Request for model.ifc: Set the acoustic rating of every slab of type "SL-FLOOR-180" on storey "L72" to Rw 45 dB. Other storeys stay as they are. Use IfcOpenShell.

First a look at what the model holds.

```python
import ifcopenshell
import ifcopenshell.util.element

model = ifcopenshell.open("model.ifc")
print(model.schema)
storey = next(s for s in model.by_type("IfcBuildingStorey") if s.Name == "L72")
slabs = [e for e in ifcopenshell.util.element.get_decomposition(storey) if e.is_a("IfcSlab")]
seen = {}
for e in slabs:
    element_type = ifcopenshell.util.element.get_type(e)
    key = (element_type.Name if element_type != e and element_type else None, ifcopenshell.util.element.get_pset(e, "Pset_SlabCommon", "AcousticRating"))
    seen[key] = seen.get(key, 0) + 1
for (name, value), count in sorted(seen.items(), key=str):
    print(count, "x", name, "|", value)
```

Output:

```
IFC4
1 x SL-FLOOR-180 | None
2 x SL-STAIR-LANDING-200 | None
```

```python
import ifcopenshell
import ifcopenshell.api.pset
import ifcopenshell.util.element

model = ifcopenshell.open("model.ifc")

storey = next(s for s in model.by_type("IfcBuildingStorey") if s.Name == "L72")
slabs = [e for e in ifcopenshell.util.element.get_decomposition(storey) if e.is_a("IfcSlab")]

count = 0
for e in slabs:
    element_type = ifcopenshell.util.element.get_type(e)
    if element_type in (None, e) or element_type.Name != "SL-FLOOR-180":
        continue
    # add_pset returns the element's existing set when there is one.
    pset = ifcopenshell.api.pset.add_pset(model, product=e, name="Pset_SlabCommon")
    ifcopenshell.api.pset.edit_pset(model, pset=pset, properties={"AcousticRating": "Rw 45 dB"})
    count += 1

print(count, "slabs updated")

model.write("model_v2.ifc")
```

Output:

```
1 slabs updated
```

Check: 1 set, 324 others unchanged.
